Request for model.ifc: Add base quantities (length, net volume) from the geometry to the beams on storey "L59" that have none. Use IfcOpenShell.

First a look at what the model holds.

```python
import ifcopenshell
import ifcopenshell.util.element
import ifcopenshell.util.unit

model = ifcopenshell.open("model.ifc")
print(model.schema)
for unit_type in ("LENGTHUNIT", "AREAUNIT", "VOLUMEUNIT"):
    print(unit_type, ifcopenshell.util.unit.calculate_unit_scale(model, unit_type))
storey = next(s for s in model.by_type("IfcBuildingStorey") if s.Name == "L59")
beams = [e for e in ifcopenshell.util.element.get_decomposition(storey) if e.is_a("IfcBeam")]
for e in sorted(beams, key=lambda e: e.id()):
    print(e.id(), e.is_a(), e.Name, list(ifcopenshell.util.element.get_psets(e, qtos_only=True)), sep=" | ")
```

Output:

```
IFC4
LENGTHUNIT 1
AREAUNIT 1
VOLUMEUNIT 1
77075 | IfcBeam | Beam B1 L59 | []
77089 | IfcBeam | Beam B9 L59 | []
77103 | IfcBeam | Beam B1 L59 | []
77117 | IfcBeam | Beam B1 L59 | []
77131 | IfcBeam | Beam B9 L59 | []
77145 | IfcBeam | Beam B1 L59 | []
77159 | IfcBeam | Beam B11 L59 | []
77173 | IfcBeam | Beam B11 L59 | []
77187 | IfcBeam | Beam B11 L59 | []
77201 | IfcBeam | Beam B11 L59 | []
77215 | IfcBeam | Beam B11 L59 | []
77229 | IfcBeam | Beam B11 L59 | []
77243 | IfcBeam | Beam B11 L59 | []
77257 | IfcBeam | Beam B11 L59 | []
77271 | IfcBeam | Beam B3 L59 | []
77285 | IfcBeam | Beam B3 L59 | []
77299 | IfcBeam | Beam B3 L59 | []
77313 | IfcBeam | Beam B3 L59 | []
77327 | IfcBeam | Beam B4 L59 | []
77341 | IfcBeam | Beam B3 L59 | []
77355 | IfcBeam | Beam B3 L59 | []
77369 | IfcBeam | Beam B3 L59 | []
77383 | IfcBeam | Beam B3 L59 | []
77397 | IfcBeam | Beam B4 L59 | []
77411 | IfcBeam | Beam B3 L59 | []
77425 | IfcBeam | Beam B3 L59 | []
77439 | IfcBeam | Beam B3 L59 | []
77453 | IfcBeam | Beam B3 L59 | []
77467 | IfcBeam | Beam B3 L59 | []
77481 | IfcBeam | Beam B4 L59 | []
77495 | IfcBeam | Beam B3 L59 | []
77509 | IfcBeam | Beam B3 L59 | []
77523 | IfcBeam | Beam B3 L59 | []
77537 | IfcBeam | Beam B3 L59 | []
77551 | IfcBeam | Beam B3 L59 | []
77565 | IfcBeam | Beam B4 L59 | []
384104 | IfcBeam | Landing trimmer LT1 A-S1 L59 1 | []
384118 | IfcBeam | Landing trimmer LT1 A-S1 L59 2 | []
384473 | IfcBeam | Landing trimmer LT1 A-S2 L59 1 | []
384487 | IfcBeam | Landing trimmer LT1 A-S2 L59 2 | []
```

```python
import ifcopenshell
import ifcopenshell.api.pset
import ifcopenshell.geom
import ifcopenshell.util.element
import ifcopenshell.util.shape
import ifcopenshell.util.unit

model = ifcopenshell.open("model.ifc")
unit_scale = ifcopenshell.util.unit.calculate_unit_scale(model)
volume_scale = ifcopenshell.util.unit.calculate_unit_scale(model, "VOLUMEUNIT")
settings = ifcopenshell.geom.settings()

storey = next(s for s in model.by_type("IfcBuildingStorey") if s.Name == "L59")
beams = [e for e in ifcopenshell.util.element.get_decomposition(storey) if e.is_a("IfcBeam")]

for e in sorted(beams, key=lambda e: e.id()):
    if ifcopenshell.util.element.get_psets(e, qtos_only=True, should_inherit=False):
        continue
    # Geometry comes back in metres, in the element's own axes.
    shape = ifcopenshell.geom.create_shape(settings, e)
    values = {
        "Length": ifcopenshell.util.shape.get_max_xyz(shape.geometry) / unit_scale,
        "NetVolume": ifcopenshell.util.shape.get_volume(shape.geometry) / volume_scale,
    }
    qto = ifcopenshell.api.pset.add_qto(model, product=e, name="Qto_BeamBaseQuantities")
    ifcopenshell.api.pset.edit_qto(model, qto=qto, properties=values)
    print(e.id(), {k: round(v, 3) for k, v in values.items()})

model.write("model_v2.ifc")
```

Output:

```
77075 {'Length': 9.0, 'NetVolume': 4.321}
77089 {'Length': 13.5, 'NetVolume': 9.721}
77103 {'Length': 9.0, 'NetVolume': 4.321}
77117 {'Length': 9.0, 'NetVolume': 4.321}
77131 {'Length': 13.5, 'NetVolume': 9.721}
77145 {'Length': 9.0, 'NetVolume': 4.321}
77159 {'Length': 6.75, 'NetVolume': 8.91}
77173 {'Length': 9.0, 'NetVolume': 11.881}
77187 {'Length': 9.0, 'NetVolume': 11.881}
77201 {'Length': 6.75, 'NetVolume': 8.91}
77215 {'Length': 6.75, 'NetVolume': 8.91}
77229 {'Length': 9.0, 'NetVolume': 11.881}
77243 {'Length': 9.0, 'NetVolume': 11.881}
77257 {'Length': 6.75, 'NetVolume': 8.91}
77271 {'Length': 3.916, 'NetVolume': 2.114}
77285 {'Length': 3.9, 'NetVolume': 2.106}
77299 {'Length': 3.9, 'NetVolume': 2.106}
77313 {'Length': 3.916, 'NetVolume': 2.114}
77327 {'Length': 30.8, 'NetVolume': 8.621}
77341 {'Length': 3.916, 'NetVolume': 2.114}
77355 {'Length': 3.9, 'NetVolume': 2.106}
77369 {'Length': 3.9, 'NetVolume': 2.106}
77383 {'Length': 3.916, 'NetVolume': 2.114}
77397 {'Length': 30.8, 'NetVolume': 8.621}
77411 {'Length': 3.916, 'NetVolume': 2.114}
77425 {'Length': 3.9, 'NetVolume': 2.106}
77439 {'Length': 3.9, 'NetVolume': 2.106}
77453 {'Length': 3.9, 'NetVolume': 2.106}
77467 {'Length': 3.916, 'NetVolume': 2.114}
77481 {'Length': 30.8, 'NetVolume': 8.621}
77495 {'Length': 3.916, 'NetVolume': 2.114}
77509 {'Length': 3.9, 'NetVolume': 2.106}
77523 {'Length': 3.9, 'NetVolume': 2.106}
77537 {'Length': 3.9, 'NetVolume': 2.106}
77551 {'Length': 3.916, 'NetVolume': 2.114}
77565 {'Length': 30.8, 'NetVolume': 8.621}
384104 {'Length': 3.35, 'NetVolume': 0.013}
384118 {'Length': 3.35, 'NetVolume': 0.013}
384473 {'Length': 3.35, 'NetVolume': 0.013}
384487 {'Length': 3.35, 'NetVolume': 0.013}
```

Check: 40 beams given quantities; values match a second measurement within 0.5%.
